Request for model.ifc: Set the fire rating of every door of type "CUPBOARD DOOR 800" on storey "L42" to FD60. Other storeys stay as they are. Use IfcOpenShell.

First a look at what the model holds.

```python
import ifcopenshell
import ifcopenshell.util.element

model = ifcopenshell.open("model.ifc")
print(model.schema)
storey = next(s for s in model.by_type("IfcBuildingStorey") if s.Name == "L42")
doors = [e for e in ifcopenshell.util.element.get_decomposition(storey) if e.is_a("IfcDoor")]
seen = {}
for e in doors:
    element_type = ifcopenshell.util.element.get_type(e)
    key = (element_type.Name if element_type != e and element_type else None, ifcopenshell.util.element.get_pset(e, "Pset_DoorCommon", "FireRating"))
    seen[key] = seen.get(key, 0) + 1
for (name, value), count in sorted(seen.items(), key=str):
    print(count, "x", name, "|", value)
```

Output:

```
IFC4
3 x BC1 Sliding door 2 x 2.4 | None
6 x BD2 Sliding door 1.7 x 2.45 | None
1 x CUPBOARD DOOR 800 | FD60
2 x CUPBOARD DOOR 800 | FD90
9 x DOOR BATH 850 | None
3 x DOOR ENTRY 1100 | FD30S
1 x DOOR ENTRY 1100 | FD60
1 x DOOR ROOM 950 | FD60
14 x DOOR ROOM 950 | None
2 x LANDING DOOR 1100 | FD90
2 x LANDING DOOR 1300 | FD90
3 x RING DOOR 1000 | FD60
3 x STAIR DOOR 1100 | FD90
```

```python
import ifcopenshell
import ifcopenshell.api.pset
import ifcopenshell.util.element

model = ifcopenshell.open("model.ifc")

storey = next(s for s in model.by_type("IfcBuildingStorey") if s.Name == "L42")
doors = [e for e in ifcopenshell.util.element.get_decomposition(storey) if e.is_a("IfcDoor")]

count = 0
for e in doors:
    element_type = ifcopenshell.util.element.get_type(e)
    if element_type in (None, e) or element_type.Name != "CUPBOARD DOOR 800":
        continue
    found = ifcopenshell.util.element.get_pset(e, "Pset_DoorCommon", should_inherit=False)
    if found:
        pset = model.by_id(found["id"])
        if len(ifcopenshell.util.element.get_elements_by_pset(pset)) > 1:
            pset = ifcopenshell.api.pset.unshare_pset(model, products=[e], pset=pset)[0]
    else:
        pset = ifcopenshell.api.pset.add_pset(model, product=e, name="Pset_DoorCommon")
    ifcopenshell.api.pset.edit_pset(model, pset=pset, properties={"FireRating": "FD60"})
    count += 1

print(count, "doors updated")

model.write("model_updated.ifc")
```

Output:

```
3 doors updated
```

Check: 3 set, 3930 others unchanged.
